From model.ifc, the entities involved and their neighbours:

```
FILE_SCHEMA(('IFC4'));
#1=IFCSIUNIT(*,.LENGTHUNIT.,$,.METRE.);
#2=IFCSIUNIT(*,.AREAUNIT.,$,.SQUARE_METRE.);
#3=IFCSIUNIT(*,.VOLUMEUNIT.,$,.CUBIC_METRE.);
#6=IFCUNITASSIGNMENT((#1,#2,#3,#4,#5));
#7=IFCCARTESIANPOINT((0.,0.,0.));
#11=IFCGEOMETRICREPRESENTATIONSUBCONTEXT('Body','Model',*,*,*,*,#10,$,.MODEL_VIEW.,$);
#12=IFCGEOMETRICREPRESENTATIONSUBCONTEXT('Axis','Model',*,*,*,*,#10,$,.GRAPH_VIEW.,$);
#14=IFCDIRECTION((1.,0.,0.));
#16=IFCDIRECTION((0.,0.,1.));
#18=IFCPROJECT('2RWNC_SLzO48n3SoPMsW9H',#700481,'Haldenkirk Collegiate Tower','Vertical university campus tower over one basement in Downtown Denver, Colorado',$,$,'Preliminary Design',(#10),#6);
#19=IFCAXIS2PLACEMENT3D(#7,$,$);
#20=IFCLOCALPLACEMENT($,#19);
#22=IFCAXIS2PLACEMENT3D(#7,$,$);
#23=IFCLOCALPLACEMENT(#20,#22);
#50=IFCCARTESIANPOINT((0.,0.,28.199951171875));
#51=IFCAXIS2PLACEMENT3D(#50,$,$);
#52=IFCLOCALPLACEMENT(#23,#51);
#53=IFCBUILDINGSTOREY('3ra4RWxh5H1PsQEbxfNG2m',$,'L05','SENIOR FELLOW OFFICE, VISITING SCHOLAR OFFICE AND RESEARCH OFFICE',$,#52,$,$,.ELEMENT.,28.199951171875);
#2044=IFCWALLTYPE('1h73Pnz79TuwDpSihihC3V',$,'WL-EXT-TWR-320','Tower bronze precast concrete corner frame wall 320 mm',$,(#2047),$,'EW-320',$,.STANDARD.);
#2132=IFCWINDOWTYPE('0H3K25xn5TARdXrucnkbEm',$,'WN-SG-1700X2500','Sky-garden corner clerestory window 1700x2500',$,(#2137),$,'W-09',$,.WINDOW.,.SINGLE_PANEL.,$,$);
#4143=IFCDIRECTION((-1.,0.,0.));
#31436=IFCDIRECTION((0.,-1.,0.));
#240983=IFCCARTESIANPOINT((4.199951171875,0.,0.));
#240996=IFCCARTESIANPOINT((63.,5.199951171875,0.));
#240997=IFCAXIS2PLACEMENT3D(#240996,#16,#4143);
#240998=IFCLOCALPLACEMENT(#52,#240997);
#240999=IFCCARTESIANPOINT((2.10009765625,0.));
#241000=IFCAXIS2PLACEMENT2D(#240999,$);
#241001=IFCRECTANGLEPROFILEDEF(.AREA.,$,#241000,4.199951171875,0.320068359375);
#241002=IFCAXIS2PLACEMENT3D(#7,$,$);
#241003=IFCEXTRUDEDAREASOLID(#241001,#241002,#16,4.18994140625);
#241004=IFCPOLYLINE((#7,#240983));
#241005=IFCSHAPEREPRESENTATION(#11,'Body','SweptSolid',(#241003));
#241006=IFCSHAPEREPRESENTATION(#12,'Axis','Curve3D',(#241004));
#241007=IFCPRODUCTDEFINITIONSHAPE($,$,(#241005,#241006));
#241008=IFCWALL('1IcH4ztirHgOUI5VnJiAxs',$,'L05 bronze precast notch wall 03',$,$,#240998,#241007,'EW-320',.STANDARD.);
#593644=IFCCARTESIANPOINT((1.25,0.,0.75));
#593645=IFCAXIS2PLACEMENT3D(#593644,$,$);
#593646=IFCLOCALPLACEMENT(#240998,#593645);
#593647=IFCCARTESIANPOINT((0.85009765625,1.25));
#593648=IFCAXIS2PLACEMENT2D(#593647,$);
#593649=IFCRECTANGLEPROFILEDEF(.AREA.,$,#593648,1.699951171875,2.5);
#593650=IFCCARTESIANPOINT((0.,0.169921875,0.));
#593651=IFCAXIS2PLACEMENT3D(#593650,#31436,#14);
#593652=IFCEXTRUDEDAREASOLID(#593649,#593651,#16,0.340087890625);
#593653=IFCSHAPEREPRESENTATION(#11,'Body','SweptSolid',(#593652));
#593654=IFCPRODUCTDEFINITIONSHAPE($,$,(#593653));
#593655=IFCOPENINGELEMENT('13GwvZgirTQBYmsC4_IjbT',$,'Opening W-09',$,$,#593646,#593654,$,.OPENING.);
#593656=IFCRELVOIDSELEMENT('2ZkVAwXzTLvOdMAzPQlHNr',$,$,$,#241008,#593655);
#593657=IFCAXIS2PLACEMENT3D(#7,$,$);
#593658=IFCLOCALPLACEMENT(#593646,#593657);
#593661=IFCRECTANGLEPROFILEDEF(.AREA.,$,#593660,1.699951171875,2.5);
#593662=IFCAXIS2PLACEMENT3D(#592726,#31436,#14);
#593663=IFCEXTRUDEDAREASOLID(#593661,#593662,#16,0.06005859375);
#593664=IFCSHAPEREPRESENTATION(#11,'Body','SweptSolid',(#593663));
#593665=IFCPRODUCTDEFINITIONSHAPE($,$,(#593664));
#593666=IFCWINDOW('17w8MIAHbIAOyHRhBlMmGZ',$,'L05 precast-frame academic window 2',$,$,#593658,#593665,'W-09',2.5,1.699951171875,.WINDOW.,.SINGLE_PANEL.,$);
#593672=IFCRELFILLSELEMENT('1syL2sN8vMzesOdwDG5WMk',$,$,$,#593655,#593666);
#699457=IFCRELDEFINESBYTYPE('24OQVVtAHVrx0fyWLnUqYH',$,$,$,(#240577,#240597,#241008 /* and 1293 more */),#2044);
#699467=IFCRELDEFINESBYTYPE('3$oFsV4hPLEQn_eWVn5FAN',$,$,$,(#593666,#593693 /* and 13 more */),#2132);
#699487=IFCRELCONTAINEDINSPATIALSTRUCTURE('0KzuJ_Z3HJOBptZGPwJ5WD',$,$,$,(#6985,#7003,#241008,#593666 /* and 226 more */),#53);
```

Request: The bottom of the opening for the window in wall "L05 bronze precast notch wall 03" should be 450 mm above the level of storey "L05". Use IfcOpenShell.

```python
import numpy as np
import ifcopenshell
import ifcopenshell.api.geometry
import ifcopenshell.geom
import ifcopenshell.util.element
import ifcopenshell.util.placement
import ifcopenshell.util.shape
import ifcopenshell.util.unit

model = ifcopenshell.open("model.ifc")
unit_scale = ifcopenshell.util.unit.calculate_unit_scale(model)

window = model.by_guid("17w8MIAHbIAOyHRhBlMmGZ")
opening = window.FillsVoids[0].RelatingOpeningElement
storey = ifcopenshell.util.element.get_container(window, ifc_class="IfcBuildingStorey")
level = ifcopenshell.util.placement.get_local_placement(storey.ObjectPlacement)[2, 3]

# The opening's origin need not be at the sill, so measure its lowest point.
shape = ifcopenshell.geom.create_shape(ifcopenshell.geom.settings(), opening)
bottom = ifcopenshell.util.shape.get_shape_bottom_elevation(shape, shape.geometry) / unit_scale
dz = level + 0.45 - bottom

shift = np.array([0.0, 0.0, dz])
# The window is placed relative to its opening, so it follows when the opening moves.
matrix = ifcopenshell.util.placement.get_local_placement(opening.ObjectPlacement)
matrix[:3, 3] += shift
ifcopenshell.api.geometry.edit_object_placement(
    model, product=opening, matrix=matrix, is_si=False, should_transform_children=True
)

print(f"moved by {dz * unit_scale:+.3f} m")

model.write("model_v2.ifc")
```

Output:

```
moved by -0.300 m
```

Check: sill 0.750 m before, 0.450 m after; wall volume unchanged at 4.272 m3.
